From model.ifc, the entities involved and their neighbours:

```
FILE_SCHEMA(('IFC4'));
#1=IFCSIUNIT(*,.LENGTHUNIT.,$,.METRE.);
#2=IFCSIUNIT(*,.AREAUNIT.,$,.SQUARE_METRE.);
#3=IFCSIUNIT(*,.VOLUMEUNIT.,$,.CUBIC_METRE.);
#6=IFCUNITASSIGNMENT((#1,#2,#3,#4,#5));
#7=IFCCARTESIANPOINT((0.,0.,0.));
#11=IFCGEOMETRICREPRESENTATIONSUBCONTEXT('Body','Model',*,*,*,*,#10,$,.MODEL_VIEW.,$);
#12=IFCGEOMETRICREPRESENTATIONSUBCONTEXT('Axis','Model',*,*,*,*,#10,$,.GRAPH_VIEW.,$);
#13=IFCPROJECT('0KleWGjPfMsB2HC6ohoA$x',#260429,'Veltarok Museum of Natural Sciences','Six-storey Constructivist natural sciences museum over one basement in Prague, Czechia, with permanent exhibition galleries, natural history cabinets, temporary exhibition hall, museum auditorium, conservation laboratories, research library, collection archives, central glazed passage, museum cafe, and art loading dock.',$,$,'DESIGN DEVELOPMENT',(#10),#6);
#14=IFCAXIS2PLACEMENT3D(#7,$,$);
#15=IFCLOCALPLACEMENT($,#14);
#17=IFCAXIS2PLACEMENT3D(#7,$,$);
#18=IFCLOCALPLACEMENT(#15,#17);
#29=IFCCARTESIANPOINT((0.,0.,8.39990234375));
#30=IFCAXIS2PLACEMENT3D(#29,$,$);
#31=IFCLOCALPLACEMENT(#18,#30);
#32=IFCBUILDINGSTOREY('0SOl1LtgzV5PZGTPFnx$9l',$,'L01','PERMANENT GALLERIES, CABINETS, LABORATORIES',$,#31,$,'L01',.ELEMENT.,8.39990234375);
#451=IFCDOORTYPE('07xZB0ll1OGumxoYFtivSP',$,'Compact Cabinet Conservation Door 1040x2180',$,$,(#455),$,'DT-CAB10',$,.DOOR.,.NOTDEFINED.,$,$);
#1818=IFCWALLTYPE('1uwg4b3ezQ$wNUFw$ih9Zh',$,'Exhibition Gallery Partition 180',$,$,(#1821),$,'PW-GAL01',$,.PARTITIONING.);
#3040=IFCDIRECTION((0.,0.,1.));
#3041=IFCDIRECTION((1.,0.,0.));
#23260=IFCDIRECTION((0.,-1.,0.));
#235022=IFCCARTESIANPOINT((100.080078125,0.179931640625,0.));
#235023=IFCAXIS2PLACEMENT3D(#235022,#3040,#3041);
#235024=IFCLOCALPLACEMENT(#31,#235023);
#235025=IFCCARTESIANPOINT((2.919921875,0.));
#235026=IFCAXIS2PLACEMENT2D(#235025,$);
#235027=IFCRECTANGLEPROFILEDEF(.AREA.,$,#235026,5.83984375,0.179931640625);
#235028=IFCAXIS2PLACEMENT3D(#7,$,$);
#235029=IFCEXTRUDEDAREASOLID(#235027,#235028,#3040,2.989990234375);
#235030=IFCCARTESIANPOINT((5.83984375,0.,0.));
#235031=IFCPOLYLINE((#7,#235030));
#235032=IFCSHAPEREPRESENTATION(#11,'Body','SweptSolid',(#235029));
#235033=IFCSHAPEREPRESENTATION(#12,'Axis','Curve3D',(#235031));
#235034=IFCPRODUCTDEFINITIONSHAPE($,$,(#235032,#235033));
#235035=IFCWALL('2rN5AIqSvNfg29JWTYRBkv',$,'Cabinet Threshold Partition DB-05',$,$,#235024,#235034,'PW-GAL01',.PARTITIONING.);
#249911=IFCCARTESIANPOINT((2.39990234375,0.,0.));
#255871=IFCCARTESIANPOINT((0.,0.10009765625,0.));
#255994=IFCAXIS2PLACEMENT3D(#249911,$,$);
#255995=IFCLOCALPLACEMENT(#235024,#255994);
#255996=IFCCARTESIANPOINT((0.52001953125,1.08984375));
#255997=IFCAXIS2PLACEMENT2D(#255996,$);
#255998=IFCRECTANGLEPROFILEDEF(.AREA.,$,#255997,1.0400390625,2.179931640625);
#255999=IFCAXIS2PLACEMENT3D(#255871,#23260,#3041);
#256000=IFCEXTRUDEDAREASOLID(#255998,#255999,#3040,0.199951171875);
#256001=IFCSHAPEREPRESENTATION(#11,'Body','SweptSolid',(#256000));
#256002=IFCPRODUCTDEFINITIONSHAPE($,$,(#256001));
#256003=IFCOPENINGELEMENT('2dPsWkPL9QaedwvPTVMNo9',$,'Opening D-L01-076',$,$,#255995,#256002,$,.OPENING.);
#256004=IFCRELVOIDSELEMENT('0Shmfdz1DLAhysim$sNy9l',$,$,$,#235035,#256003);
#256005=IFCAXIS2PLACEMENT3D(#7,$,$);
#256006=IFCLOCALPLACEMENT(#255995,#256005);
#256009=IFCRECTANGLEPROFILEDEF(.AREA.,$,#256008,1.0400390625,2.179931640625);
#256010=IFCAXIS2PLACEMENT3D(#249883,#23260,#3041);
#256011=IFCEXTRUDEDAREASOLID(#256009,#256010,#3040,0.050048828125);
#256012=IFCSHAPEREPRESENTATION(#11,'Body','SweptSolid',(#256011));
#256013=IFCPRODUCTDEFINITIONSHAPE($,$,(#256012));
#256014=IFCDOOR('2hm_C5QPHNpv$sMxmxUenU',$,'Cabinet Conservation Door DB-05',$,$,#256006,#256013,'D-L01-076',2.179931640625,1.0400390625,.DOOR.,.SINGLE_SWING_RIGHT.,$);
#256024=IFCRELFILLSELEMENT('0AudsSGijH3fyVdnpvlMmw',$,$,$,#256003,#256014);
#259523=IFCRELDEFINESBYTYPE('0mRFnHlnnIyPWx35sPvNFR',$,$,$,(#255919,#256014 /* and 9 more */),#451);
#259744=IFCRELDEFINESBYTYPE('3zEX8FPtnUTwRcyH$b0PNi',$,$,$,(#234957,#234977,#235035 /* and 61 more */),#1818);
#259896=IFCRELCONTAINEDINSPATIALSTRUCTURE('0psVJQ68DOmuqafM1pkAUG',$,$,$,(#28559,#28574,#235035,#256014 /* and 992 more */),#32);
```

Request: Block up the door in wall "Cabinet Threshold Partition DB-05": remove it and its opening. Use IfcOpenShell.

```python
import ifcopenshell
import ifcopenshell.api.feature
import ifcopenshell.api.root
import ifcopenshell.geom
import ifcopenshell.util.shape

model = ifcopenshell.open("model.ifc")
settings = ifcopenshell.geom.settings()


def volume(element):
    """Net volume in cubic metres, openings subtracted."""
    shape = ifcopenshell.geom.create_shape(settings, element)
    return ifcopenshell.util.shape.get_volume(shape.geometry)


door = model.by_id(256014)
opening = door.FillsVoids[0].RelatingOpeningElement
wall = opening.VoidsElements[0].RelatingBuildingElement
before = volume(wall)

ifcopenshell.api.root.remove_product(model, product=door)
ifcopenshell.api.feature.remove_feature(model, feature=opening)

after = volume(wall)

print(f"wall volume {before:.3f} -> {after:.3f} m3")

model.write("model_updated.ifc")
```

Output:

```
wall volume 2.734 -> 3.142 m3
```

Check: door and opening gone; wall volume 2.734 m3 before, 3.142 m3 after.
